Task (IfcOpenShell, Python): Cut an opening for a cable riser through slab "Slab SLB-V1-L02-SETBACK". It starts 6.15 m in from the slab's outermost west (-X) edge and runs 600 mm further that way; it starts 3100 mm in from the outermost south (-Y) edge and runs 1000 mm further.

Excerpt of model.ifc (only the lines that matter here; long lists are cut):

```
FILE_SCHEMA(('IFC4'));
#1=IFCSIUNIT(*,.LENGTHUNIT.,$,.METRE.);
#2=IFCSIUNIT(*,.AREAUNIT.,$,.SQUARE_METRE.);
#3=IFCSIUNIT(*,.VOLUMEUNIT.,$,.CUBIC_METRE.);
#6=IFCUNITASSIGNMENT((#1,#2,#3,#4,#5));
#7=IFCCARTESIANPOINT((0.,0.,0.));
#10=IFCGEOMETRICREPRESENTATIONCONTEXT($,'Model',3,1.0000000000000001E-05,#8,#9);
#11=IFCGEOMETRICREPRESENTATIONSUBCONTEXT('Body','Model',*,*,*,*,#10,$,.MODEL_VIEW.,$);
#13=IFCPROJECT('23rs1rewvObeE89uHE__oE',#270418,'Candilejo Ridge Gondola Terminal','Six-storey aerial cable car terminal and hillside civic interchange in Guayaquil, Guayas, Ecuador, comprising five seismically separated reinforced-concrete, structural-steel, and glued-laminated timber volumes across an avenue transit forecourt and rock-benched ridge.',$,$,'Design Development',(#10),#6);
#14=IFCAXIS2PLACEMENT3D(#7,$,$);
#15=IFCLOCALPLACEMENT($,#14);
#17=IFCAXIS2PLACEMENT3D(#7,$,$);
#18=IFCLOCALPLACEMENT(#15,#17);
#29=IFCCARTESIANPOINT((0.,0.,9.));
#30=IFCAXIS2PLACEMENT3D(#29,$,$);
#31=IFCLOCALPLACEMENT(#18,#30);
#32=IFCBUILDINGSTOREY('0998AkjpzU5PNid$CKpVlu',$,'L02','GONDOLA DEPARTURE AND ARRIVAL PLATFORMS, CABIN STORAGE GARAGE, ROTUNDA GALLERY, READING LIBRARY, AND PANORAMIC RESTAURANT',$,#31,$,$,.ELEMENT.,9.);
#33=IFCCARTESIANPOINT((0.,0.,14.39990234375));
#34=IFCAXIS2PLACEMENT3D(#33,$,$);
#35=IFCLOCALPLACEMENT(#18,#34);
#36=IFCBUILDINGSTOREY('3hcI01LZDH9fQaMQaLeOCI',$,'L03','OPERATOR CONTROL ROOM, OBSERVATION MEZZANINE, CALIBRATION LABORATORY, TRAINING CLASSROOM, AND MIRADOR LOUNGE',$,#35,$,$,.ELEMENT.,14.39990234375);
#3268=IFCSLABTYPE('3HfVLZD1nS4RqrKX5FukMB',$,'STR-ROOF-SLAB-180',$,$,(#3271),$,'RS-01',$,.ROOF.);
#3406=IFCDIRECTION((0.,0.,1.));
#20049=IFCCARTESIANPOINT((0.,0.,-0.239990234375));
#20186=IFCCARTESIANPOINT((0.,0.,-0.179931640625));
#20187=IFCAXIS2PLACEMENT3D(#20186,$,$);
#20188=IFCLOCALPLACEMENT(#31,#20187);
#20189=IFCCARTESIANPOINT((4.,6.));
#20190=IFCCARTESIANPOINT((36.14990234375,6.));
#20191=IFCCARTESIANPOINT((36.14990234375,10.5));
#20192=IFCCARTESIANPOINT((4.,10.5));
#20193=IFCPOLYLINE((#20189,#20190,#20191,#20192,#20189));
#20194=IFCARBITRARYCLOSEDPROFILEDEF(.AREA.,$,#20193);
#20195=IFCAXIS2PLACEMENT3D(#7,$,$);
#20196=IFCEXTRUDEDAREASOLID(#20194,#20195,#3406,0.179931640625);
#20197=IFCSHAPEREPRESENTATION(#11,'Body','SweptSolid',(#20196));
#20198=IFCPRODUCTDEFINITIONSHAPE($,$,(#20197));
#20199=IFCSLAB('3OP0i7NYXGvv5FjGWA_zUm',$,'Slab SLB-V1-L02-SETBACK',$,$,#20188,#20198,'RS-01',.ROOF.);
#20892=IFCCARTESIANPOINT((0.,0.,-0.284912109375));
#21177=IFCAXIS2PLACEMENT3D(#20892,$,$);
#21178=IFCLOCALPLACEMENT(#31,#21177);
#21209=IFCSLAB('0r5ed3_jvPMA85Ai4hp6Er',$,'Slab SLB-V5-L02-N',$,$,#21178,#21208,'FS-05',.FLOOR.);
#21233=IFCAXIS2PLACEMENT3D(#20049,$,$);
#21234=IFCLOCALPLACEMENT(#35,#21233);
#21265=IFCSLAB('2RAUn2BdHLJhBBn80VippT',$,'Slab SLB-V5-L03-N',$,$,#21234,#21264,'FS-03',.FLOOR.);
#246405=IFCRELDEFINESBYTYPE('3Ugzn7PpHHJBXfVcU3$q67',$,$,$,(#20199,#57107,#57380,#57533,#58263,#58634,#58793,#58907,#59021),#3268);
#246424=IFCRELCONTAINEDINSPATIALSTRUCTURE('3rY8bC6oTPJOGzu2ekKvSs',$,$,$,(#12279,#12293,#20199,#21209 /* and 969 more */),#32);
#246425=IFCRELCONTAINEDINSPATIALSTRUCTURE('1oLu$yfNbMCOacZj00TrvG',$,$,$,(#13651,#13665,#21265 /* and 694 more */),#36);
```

```python
import numpy as np
import ifcopenshell
import ifcopenshell.api.feature
import ifcopenshell.api.geometry
import ifcopenshell.api.root
import ifcopenshell.geom
import ifcopenshell.util.placement
import ifcopenshell.util.representation
import ifcopenshell.util.shape
import ifcopenshell.util.unit

model = ifcopenshell.open("model.ifc")
unit_scale = ifcopenshell.util.unit.calculate_unit_scale(model)
settings = ifcopenshell.geom.settings()


def volume(element):
    """Net volume in cubic metres, openings subtracted."""
    shape = ifcopenshell.geom.create_shape(settings, element)
    return ifcopenshell.util.shape.get_volume(shape.geometry)


slab = model.by_guid("3OP0i7NYXGvv5FjGWA_zUm")
before = volume(slab)

# Extent in the slab's own axes, in metres. The edges named are its -X and -Y sides.
slab_shape = ifcopenshell.geom.create_shape(settings, slab)
vertices = ifcopenshell.util.shape.get_vertices(slab_shape.geometry)
x_min, y_min, bottom = vertices.min(axis=0)
top = vertices[:, 2].max()

opening = ifcopenshell.api.root.create_entity(model, ifc_class="IfcOpeningElement", name="Cable riser opening", predefined_type="OPENING")
context = ifcopenshell.util.representation.get_context(model, "Model", "Body", "MODEL_VIEW")
width, depth = 0.6, 1
outline = [(0.0, 0.0), (width, 0.0), (width, depth), (0.0, depth), (0.0, 0.0)]
# Overshoot both faces by 50 mm so the cut is clean.
shape = ifcopenshell.api.geometry.add_slab_representation(
    model, context=context, depth=top - bottom + 0.1, polyline=outline
)
ifcopenshell.api.geometry.assign_representation(model, product=opening, representation=shape)

matrix = ifcopenshell.util.placement.get_local_placement(slab.ObjectPlacement)
matrix[:, 3] = matrix @ np.append(np.array([x_min + 6.15, y_min + 3.1, bottom - 0.05]) / unit_scale, 1.0)
ifcopenshell.api.geometry.edit_object_placement(model, product=opening, matrix=matrix, is_si=False)
ifcopenshell.api.feature.add_feature(model, feature=opening, element=slab)

after = volume(slab)

print(f"slab volume {before:.3f} -> {after:.3f} m3")

model.write("model_updated.ifc")
```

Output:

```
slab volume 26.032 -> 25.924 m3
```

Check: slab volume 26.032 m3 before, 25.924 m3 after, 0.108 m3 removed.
